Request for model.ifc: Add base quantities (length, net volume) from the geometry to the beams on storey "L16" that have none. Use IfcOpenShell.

First a look at what the model holds.

```python
import ifcopenshell
import ifcopenshell.util.element
import ifcopenshell.util.unit

model = ifcopenshell.open("model.ifc")
print(model.schema)
for unit_type in ("LENGTHUNIT", "AREAUNIT", "VOLUMEUNIT"):
    print(unit_type, ifcopenshell.util.unit.calculate_unit_scale(model, unit_type))
storey = next(s for s in model.by_type("IfcBuildingStorey") if s.Name == "L16")
beams = [e for e in ifcopenshell.util.element.get_decomposition(storey) if e.is_a("IfcBeam")]
for e in sorted(beams, key=lambda e: e.id()):
    print(e.id(), e.is_a(), e.Name, list(ifcopenshell.util.element.get_psets(e, qtos_only=True)), sep=" | ")
```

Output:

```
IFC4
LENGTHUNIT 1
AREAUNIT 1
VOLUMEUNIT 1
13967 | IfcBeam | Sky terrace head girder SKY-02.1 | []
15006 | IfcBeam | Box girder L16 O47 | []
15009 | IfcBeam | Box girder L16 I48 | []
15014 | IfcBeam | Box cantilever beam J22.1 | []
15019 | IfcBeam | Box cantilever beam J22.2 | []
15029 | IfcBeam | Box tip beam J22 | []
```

```python
import ifcopenshell
import ifcopenshell.api.pset
import ifcopenshell.geom
import ifcopenshell.util.element
import ifcopenshell.util.shape
import ifcopenshell.util.unit

model = ifcopenshell.open("model.ifc")
unit_scale = ifcopenshell.util.unit.calculate_unit_scale(model)
volume_scale = ifcopenshell.util.unit.calculate_unit_scale(model, "VOLUMEUNIT")
settings = ifcopenshell.geom.settings()

storey = next(s for s in model.by_type("IfcBuildingStorey") if s.Name == "L16")
beams = [e for e in ifcopenshell.util.element.get_decomposition(storey) if e.is_a("IfcBeam")]

for e in sorted(beams, key=lambda e: e.id()):
    if ifcopenshell.util.element.get_psets(e, qtos_only=True, should_inherit=False):
        continue
    # Geometry comes back in metres, in the element's own axes.
    shape = ifcopenshell.geom.create_shape(settings, e)
    values = {
        "Length": ifcopenshell.util.shape.get_max_xyz(shape.geometry) / unit_scale,
        "NetVolume": ifcopenshell.util.shape.get_volume(shape.geometry) / volume_scale,
    }
    qto = ifcopenshell.api.pset.add_qto(model, product=e, name="Qto_BeamBaseQuantities")
    ifcopenshell.api.pset.edit_qto(model, qto=qto, properties=values)
    print(e.id(), {k: round(v, 3) for k, v in values.items()})

model.write("model_edited.ifc")
```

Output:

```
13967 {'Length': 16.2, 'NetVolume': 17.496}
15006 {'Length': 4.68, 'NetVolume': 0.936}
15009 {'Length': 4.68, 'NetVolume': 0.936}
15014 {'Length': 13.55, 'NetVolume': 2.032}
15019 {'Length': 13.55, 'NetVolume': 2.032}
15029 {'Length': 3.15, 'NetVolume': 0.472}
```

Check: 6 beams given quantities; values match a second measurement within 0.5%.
